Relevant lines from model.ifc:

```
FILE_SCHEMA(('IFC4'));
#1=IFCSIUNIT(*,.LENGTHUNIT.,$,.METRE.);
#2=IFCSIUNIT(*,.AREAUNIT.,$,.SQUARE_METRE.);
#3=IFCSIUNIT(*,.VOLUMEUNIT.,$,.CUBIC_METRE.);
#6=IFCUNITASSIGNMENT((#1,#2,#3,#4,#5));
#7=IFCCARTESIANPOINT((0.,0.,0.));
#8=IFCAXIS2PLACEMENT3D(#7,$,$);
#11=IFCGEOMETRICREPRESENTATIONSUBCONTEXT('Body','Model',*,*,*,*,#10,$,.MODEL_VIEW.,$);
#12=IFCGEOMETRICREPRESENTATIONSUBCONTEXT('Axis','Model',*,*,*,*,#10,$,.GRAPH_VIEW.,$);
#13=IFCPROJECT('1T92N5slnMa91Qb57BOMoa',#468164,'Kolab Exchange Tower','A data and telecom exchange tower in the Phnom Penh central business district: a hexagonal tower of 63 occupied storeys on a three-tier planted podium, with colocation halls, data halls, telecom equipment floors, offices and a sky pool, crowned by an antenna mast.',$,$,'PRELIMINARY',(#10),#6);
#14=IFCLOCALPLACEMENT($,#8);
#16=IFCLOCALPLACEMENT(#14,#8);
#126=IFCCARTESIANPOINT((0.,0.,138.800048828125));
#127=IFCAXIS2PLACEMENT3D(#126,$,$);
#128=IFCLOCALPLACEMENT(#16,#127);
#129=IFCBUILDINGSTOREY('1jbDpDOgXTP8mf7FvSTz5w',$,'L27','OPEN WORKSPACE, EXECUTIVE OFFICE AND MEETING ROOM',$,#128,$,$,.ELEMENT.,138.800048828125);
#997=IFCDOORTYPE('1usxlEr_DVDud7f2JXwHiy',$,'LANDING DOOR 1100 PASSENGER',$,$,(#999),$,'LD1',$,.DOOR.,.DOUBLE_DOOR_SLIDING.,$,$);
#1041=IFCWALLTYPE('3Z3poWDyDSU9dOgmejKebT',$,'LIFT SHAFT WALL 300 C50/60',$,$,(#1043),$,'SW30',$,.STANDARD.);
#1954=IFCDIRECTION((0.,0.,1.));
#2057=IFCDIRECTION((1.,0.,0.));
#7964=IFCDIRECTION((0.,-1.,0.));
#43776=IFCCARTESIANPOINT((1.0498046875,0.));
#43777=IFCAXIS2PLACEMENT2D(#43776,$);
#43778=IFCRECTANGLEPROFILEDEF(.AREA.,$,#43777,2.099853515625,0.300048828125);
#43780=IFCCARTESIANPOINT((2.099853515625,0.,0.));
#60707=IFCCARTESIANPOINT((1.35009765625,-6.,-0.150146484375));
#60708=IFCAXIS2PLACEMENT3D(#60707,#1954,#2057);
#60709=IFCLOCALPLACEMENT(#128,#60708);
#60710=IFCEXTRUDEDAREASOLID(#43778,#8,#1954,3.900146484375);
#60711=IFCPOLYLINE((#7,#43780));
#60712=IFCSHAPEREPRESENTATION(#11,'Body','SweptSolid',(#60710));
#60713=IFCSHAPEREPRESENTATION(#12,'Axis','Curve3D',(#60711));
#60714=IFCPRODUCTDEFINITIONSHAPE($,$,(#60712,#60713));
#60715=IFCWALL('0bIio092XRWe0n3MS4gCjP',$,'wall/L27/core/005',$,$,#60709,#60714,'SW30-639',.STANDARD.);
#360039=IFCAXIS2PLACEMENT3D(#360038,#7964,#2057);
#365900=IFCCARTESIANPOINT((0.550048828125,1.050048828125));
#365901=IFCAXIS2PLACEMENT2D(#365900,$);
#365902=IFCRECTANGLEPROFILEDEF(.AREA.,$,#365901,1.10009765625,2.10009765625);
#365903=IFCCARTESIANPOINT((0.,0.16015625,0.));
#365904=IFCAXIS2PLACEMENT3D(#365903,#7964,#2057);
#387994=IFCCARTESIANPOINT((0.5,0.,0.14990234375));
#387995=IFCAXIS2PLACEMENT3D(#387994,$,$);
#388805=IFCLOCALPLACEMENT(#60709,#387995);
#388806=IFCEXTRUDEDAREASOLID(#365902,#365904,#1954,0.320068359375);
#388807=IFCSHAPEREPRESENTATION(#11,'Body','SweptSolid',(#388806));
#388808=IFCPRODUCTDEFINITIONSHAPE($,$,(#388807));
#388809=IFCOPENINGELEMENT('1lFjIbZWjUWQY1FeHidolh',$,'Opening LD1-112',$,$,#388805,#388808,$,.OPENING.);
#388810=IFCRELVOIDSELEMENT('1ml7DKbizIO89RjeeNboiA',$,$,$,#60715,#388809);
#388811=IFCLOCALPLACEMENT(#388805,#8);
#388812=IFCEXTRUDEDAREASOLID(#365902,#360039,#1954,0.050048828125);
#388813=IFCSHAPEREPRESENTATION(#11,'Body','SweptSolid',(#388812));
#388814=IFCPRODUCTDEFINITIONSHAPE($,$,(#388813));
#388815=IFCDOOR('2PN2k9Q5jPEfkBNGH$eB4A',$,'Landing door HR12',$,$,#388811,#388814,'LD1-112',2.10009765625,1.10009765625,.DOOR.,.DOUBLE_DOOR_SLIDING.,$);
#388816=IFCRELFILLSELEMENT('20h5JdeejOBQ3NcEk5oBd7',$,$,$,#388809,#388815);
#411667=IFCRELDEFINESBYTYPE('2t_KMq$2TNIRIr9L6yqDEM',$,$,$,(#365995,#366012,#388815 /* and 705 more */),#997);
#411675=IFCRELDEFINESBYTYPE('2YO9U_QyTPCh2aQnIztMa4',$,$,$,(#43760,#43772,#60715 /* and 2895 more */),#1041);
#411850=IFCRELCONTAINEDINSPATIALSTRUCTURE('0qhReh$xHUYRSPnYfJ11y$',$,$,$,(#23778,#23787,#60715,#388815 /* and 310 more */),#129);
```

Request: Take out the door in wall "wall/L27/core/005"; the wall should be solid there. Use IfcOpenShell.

```python
import ifcopenshell
import ifcopenshell.api.feature
import ifcopenshell.api.root
import ifcopenshell.geom
import ifcopenshell.util.shape

model = ifcopenshell.open("model.ifc")
settings = ifcopenshell.geom.settings()


def volume(element):
    """Net volume in cubic metres, openings subtracted."""
    shape = ifcopenshell.geom.create_shape(settings, element)
    return ifcopenshell.util.shape.get_volume(shape.geometry)


door = model.by_id(388815)
opening = door.FillsVoids[0].RelatingOpeningElement
wall = opening.VoidsElements[0].RelatingBuildingElement
before = volume(wall)

ifcopenshell.api.root.remove_product(model, product=door)
ifcopenshell.api.feature.remove_feature(model, feature=opening)

after = volume(wall)

print(f"wall volume {before:.3f} -> {after:.3f} m3")

model.write("model_edited.ifc")
```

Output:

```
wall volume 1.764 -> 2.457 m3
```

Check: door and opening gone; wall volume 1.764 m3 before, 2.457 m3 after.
